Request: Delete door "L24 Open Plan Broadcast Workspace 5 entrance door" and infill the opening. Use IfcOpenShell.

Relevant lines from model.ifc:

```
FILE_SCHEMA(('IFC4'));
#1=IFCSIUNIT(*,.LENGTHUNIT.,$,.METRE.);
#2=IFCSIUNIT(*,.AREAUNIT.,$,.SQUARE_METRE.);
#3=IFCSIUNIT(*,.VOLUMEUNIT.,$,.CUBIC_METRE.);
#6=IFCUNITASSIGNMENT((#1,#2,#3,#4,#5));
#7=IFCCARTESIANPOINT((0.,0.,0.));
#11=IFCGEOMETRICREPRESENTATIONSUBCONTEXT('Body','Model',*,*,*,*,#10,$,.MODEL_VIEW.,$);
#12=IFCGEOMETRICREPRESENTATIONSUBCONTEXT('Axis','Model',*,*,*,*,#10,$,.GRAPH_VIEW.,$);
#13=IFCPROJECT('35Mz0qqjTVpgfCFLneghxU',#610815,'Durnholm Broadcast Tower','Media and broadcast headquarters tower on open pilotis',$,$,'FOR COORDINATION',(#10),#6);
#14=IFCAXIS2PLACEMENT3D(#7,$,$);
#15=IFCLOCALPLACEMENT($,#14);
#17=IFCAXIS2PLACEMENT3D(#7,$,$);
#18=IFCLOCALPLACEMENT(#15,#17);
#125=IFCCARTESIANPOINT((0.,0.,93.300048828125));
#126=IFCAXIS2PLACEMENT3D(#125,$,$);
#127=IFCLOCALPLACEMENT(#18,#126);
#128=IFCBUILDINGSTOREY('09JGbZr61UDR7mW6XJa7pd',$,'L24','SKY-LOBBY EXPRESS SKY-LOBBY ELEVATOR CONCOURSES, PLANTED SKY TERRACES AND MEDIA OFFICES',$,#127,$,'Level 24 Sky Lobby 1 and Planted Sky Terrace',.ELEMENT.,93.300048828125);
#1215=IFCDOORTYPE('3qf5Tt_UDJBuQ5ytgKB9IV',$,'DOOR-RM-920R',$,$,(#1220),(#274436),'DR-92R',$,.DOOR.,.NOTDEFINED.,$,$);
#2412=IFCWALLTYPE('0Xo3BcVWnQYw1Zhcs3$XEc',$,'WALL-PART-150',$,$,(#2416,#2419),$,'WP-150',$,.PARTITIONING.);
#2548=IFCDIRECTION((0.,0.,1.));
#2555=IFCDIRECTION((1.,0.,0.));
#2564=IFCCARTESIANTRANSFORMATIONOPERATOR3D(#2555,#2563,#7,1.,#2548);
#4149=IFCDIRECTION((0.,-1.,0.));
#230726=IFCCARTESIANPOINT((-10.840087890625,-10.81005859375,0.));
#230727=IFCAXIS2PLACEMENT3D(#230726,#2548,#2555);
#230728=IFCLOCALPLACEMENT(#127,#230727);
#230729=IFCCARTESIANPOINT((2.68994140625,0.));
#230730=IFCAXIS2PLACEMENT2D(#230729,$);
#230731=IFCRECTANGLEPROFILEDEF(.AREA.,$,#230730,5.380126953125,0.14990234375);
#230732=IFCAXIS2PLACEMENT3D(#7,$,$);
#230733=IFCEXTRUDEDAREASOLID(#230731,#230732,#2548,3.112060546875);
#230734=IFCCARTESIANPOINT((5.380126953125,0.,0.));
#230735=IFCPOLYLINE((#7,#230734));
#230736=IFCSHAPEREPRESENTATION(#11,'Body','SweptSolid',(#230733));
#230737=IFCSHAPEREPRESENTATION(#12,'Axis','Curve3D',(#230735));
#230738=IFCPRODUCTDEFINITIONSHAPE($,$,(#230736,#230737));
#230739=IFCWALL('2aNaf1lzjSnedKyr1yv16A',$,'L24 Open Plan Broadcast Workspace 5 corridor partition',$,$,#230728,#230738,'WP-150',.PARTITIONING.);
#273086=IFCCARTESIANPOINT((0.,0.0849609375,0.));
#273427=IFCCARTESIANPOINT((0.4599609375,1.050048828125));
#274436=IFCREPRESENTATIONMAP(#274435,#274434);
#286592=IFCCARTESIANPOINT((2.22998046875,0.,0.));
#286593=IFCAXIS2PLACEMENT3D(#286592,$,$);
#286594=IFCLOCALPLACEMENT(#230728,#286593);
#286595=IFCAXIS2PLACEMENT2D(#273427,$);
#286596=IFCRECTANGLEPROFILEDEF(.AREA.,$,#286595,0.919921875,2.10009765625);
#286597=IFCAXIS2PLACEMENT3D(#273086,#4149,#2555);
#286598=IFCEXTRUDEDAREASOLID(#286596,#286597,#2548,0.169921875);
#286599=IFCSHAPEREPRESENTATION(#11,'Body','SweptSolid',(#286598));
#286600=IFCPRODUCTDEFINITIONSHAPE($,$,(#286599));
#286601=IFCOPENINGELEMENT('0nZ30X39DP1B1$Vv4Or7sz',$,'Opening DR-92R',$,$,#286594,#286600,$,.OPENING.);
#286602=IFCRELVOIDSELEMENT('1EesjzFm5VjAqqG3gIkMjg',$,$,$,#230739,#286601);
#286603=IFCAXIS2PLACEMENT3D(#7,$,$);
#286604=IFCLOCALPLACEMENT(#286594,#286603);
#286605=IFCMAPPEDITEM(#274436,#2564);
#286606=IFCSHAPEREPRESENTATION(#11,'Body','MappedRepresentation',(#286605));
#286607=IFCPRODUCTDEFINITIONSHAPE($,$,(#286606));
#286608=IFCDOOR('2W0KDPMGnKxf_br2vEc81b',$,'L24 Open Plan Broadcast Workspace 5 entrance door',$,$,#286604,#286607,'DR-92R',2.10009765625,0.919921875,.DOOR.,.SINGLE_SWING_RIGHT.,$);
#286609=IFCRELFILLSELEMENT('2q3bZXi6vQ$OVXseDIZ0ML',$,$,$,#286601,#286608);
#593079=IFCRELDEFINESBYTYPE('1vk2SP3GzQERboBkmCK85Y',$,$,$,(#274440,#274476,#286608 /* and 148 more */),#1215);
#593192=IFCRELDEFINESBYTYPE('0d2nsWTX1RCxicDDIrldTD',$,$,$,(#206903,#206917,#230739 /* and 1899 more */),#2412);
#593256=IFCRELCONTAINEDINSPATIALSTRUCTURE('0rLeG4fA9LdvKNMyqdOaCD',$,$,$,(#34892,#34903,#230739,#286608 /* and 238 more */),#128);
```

```python
import ifcopenshell
import ifcopenshell.api.feature
import ifcopenshell.api.root
import ifcopenshell.geom
import ifcopenshell.util.shape

model = ifcopenshell.open("model.ifc")
settings = ifcopenshell.geom.settings()


def volume(element):
    """Net volume in cubic metres, openings subtracted."""
    shape = ifcopenshell.geom.create_shape(settings, element)
    return ifcopenshell.util.shape.get_volume(shape.geometry)


door = model.by_id(286608)
opening = door.FillsVoids[0].RelatingOpeningElement
wall = opening.VoidsElements[0].RelatingBuildingElement
before = volume(wall)

ifcopenshell.api.root.remove_product(model, product=door)
ifcopenshell.api.feature.remove_feature(model, feature=opening)

after = volume(wall)

print(f"wall volume {before:.3f} -> {after:.3f} m3")

model.write("model-out.ifc")
```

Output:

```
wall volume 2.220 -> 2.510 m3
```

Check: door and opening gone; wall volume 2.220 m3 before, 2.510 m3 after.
